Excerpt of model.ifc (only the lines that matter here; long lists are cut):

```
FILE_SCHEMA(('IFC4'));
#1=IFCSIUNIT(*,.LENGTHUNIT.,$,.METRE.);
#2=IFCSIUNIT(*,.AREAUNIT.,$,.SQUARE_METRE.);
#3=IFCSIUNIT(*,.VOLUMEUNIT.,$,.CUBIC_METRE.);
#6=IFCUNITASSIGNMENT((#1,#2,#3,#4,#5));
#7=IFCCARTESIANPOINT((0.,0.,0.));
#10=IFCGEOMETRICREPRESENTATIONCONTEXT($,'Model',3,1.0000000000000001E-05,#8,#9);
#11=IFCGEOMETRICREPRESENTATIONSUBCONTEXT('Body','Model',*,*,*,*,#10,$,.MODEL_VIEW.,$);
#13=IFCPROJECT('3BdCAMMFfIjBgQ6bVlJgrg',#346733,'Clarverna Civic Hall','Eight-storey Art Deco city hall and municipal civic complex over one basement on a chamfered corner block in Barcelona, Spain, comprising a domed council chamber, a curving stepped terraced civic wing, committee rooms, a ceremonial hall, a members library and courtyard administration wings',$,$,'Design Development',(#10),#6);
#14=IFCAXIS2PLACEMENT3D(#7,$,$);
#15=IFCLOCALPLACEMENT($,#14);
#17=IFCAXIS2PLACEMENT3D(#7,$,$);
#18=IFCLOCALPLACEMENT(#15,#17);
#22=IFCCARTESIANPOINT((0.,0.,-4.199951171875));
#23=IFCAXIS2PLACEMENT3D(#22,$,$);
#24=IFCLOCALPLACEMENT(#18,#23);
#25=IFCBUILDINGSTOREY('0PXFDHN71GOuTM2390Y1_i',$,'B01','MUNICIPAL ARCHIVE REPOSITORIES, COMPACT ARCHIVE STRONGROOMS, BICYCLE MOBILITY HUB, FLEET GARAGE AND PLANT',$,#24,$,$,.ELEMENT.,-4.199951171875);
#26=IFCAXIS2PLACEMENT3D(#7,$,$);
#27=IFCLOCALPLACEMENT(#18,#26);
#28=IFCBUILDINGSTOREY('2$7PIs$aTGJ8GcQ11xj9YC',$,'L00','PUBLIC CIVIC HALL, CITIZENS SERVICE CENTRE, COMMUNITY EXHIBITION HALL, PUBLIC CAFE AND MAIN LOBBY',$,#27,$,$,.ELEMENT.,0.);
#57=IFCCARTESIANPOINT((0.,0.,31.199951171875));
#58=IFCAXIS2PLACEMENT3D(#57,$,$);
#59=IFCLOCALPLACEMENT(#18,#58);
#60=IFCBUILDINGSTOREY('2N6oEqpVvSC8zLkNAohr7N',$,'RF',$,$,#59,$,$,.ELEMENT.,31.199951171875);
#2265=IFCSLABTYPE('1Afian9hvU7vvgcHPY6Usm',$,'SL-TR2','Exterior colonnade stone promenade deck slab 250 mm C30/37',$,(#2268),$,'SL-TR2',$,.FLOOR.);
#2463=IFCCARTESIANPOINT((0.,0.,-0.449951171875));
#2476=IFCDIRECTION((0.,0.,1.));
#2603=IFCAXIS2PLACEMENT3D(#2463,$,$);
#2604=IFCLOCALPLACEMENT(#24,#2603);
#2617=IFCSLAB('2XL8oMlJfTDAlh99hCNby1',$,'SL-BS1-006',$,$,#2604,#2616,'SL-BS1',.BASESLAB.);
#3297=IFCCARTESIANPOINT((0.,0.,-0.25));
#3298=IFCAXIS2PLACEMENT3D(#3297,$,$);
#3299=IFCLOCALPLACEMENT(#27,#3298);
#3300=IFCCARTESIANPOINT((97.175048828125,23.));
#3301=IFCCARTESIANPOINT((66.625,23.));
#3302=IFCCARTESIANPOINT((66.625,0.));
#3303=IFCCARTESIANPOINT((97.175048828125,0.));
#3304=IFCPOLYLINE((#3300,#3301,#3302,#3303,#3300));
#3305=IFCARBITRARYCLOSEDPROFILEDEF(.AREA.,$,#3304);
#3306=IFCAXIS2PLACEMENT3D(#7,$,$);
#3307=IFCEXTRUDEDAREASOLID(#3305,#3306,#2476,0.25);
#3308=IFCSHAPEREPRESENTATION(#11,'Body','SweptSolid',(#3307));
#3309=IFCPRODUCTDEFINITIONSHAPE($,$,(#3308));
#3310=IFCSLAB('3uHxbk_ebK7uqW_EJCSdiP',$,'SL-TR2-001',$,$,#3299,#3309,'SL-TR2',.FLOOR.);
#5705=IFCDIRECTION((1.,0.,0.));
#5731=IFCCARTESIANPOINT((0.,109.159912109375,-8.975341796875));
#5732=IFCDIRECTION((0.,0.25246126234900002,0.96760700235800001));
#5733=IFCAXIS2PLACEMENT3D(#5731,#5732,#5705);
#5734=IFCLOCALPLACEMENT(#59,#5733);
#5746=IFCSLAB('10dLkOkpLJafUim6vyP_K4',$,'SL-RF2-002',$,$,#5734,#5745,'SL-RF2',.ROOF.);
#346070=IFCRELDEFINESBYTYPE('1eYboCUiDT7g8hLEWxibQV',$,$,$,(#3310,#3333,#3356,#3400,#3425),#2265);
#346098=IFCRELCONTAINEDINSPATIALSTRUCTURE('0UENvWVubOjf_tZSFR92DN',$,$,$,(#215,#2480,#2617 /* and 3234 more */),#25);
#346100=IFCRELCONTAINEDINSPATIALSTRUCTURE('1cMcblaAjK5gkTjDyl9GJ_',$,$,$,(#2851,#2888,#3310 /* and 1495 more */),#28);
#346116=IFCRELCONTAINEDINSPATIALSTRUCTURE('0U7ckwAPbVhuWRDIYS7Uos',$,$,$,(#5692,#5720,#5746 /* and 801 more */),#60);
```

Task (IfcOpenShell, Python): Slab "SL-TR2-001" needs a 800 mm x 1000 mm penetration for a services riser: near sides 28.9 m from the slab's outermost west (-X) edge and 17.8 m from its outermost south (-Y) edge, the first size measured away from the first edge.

```python
import numpy as np
import ifcopenshell
import ifcopenshell.api.feature
import ifcopenshell.api.geometry
import ifcopenshell.api.root
import ifcopenshell.geom
import ifcopenshell.util.placement
import ifcopenshell.util.representation
import ifcopenshell.util.shape
import ifcopenshell.util.unit

model = ifcopenshell.open("model.ifc")
unit_scale = ifcopenshell.util.unit.calculate_unit_scale(model)
settings = ifcopenshell.geom.settings()


def volume(element):
    """Net volume in cubic metres, openings subtracted."""
    shape = ifcopenshell.geom.create_shape(settings, element)
    return ifcopenshell.util.shape.get_volume(shape.geometry)


slab = model.by_guid("3uHxbk_ebK7uqW_EJCSdiP")
before = volume(slab)

# Extent in the slab's own axes, in metres. The edges named are its -X and -Y sides.
slab_shape = ifcopenshell.geom.create_shape(settings, slab)
vertices = ifcopenshell.util.shape.get_vertices(slab_shape.geometry)
x_min, y_min, bottom = vertices.min(axis=0)
top = vertices[:, 2].max()

opening = ifcopenshell.api.root.create_entity(model, ifc_class="IfcOpeningElement", name="Services riser opening", predefined_type="OPENING")
context = ifcopenshell.util.representation.get_context(model, "Model", "Body", "MODEL_VIEW")
width, depth = 0.8, 1
outline = [(0.0, 0.0), (width, 0.0), (width, depth), (0.0, depth), (0.0, 0.0)]
# Overshoot both faces by 50 mm so the cut is clean.
shape = ifcopenshell.api.geometry.add_slab_representation(
    model, context=context, depth=top - bottom + 0.1, polyline=outline
)
ifcopenshell.api.geometry.assign_representation(model, product=opening, representation=shape)

matrix = ifcopenshell.util.placement.get_local_placement(slab.ObjectPlacement)
matrix[:, 3] = matrix @ np.append(np.array([x_min + 28.9, y_min + 17.8, bottom - 0.05]) / unit_scale, 1.0)
ifcopenshell.api.geometry.edit_object_placement(model, product=opening, matrix=matrix, is_si=False)
ifcopenshell.api.feature.add_feature(model, feature=opening, element=slab)

after = volume(slab)

print(f"slab volume {before:.3f} -> {after:.3f} m3")

model.write("model_v2.ifc")
```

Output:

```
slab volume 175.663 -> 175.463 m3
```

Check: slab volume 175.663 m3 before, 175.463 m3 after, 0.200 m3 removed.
